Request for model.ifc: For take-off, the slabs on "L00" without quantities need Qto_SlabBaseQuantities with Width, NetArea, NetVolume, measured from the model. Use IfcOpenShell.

First a look at what the model holds.

```python
import ifcopenshell
import ifcopenshell.util.element
import ifcopenshell.util.unit

model = ifcopenshell.open("model.ifc")
print(model.schema)
for unit_type in ("LENGTHUNIT", "AREAUNIT", "VOLUMEUNIT"):
    print(unit_type, ifcopenshell.util.unit.calculate_unit_scale(model, unit_type))
storey = next(s for s in model.by_type("IfcBuildingStorey") if s.Name == "L00")
slabs = [e for e in ifcopenshell.util.element.get_decomposition(storey) if e.is_a("IfcSlab")]
for e in sorted(slabs, key=lambda e: e.id()):
    print(e.id(), e.is_a(), e.Name, list(ifcopenshell.util.element.get_psets(e, qtos_only=True)), sep=" | ")
```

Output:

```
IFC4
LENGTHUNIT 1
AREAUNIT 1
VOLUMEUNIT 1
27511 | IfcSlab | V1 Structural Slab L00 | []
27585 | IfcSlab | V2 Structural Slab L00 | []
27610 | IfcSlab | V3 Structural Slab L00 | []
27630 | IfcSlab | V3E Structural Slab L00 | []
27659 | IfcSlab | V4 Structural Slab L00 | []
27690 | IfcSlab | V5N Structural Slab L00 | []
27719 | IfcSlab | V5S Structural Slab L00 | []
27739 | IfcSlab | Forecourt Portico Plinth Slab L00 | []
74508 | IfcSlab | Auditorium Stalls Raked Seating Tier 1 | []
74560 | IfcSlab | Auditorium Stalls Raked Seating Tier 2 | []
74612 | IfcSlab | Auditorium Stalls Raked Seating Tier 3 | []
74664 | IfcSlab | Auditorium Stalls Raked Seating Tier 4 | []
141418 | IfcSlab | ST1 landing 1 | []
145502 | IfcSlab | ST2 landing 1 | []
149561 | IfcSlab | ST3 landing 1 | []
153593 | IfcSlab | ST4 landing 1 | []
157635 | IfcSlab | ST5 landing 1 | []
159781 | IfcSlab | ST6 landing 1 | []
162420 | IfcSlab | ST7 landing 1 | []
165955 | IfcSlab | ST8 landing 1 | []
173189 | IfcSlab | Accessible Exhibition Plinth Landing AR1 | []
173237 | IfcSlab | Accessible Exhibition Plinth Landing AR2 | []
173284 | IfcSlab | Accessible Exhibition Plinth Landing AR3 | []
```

```python
import ifcopenshell
import ifcopenshell.api.pset
import ifcopenshell.geom
import ifcopenshell.util.element
import ifcopenshell.util.shape
import ifcopenshell.util.unit

model = ifcopenshell.open("model.ifc")
unit_scale = ifcopenshell.util.unit.calculate_unit_scale(model)
area_scale = ifcopenshell.util.unit.calculate_unit_scale(model, "AREAUNIT")
volume_scale = ifcopenshell.util.unit.calculate_unit_scale(model, "VOLUMEUNIT")
settings = ifcopenshell.geom.settings()

storey = next(s for s in model.by_type("IfcBuildingStorey") if s.Name == "L00")
slabs = [e for e in ifcopenshell.util.element.get_decomposition(storey) if e.is_a("IfcSlab")]

for e in sorted(slabs, key=lambda e: e.id()):
    if ifcopenshell.util.element.get_psets(e, qtos_only=True, should_inherit=False):
        continue
    # Geometry comes back in metres, in the element's own axes.
    shape = ifcopenshell.geom.create_shape(settings, e)
    values = {
        "Width": ifcopenshell.util.shape.get_z(shape.geometry) / unit_scale,
        "NetArea": ifcopenshell.util.shape.get_footprint_area(shape.geometry) / area_scale,
        "NetVolume": ifcopenshell.util.shape.get_volume(shape.geometry) / volume_scale,
    }
    qto = ifcopenshell.api.pset.add_qto(model, product=e, name="Qto_SlabBaseQuantities")
    ifcopenshell.api.pset.edit_qto(model, qto=qto, properties=values)
    print(e.id(), {k: round(v, 3) for k, v in values.items()})

model.write("model-out.ifc")
```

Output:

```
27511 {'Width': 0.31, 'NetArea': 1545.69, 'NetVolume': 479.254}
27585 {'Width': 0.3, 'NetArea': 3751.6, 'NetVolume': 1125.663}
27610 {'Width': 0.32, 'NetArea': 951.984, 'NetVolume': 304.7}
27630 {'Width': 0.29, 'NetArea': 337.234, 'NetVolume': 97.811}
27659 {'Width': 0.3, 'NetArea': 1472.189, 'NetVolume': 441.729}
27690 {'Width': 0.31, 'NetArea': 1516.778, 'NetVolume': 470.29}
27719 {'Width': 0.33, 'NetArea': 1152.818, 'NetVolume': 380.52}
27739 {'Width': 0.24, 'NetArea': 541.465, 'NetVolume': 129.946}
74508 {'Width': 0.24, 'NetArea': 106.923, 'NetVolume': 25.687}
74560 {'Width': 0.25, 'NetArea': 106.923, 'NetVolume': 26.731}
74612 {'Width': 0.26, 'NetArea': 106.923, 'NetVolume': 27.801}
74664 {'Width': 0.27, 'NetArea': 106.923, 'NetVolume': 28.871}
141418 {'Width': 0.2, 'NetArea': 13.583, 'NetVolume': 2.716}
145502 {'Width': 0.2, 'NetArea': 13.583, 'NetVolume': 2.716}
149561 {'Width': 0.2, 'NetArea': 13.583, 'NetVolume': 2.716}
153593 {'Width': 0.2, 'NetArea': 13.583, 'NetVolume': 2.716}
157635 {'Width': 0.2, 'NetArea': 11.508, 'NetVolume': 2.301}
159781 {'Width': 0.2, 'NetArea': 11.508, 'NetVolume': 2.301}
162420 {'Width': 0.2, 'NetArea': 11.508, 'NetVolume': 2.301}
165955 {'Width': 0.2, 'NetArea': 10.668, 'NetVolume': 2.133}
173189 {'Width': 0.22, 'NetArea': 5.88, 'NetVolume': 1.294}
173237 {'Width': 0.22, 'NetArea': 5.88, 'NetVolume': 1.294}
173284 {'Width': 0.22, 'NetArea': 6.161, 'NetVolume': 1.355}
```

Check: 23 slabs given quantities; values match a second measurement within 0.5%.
